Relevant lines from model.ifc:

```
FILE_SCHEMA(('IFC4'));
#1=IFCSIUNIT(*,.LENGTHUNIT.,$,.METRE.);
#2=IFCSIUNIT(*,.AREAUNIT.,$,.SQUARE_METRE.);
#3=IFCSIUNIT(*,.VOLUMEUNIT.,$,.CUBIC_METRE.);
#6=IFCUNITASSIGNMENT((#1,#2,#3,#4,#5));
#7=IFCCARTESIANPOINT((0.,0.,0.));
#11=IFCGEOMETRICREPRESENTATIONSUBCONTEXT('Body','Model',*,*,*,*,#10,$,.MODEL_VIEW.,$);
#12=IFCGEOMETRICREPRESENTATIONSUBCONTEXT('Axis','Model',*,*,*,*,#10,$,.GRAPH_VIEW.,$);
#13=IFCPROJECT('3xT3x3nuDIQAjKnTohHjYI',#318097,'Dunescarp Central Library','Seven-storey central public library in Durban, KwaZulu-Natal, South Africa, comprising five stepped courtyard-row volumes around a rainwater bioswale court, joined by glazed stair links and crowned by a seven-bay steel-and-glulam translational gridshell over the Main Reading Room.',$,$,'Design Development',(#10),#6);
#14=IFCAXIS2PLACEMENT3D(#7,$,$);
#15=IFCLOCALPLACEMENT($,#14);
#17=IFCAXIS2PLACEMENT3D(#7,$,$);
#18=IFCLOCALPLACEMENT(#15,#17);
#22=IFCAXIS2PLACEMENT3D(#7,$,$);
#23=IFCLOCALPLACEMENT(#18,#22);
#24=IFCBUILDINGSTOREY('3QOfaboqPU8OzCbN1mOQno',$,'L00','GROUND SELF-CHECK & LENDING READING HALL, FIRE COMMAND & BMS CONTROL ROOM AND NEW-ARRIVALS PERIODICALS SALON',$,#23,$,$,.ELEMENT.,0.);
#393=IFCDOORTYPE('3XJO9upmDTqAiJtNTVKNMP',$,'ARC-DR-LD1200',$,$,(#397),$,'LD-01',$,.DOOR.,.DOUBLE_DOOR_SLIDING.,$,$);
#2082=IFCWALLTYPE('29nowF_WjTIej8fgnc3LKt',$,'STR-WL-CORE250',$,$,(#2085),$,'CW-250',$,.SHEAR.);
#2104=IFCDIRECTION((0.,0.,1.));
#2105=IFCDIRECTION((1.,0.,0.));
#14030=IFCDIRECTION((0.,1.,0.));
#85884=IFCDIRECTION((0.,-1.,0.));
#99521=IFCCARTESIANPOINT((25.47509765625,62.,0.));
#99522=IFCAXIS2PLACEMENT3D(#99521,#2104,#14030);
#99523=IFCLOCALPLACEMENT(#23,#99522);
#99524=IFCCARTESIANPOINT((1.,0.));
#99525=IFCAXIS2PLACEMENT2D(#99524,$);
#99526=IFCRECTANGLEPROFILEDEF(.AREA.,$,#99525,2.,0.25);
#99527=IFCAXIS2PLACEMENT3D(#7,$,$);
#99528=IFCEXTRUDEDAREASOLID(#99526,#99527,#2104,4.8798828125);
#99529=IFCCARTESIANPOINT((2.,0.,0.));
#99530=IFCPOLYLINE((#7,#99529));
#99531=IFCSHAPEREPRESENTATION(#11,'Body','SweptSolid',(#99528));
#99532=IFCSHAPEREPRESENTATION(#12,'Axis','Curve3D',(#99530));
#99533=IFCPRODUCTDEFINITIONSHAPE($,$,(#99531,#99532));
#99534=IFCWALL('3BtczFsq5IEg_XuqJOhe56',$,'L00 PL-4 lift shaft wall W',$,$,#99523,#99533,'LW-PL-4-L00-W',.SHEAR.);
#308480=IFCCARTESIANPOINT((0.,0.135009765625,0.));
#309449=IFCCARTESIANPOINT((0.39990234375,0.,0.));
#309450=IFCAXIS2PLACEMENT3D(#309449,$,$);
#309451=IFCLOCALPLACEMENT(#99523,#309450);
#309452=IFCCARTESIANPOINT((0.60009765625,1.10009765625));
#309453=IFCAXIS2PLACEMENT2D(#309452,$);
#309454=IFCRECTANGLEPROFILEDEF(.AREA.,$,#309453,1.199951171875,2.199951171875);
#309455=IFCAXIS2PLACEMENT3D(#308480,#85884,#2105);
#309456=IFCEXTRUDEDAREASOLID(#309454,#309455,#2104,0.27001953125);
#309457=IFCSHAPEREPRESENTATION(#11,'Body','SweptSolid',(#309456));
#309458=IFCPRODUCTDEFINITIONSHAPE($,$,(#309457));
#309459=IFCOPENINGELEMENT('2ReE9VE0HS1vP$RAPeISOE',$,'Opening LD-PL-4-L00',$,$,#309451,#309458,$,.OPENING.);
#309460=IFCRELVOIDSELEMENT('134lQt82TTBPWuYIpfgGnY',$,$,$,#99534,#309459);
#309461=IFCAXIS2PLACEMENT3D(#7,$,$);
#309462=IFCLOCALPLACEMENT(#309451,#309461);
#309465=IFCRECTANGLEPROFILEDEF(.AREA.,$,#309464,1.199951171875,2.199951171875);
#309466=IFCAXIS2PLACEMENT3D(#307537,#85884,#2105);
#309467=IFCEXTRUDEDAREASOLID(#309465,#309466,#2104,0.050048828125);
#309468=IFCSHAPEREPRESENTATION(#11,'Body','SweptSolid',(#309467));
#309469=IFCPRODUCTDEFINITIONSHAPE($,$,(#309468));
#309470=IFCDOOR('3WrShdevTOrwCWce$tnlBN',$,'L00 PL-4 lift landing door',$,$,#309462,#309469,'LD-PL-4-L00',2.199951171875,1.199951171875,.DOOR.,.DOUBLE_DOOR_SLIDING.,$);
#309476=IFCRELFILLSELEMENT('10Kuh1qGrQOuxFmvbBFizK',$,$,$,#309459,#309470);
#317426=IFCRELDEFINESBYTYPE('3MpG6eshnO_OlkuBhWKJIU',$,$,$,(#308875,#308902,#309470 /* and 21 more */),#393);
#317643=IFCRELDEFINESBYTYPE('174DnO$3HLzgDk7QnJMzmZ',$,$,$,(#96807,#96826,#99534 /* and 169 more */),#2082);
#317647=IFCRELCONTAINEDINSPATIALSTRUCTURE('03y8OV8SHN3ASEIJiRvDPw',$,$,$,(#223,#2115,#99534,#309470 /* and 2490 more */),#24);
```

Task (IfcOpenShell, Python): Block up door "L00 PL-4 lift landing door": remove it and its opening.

```python
import ifcopenshell
import ifcopenshell.api.feature
import ifcopenshell.api.root
import ifcopenshell.geom
import ifcopenshell.util.shape

model = ifcopenshell.open("model.ifc")
settings = ifcopenshell.geom.settings()


def volume(element):
    """Net volume in cubic metres, openings subtracted."""
    shape = ifcopenshell.geom.create_shape(settings, element)
    return ifcopenshell.util.shape.get_volume(shape.geometry)


door = model.by_guid("3WrShdevTOrwCWce$tnlBN")
opening = door.FillsVoids[0].RelatingOpeningElement
wall = opening.VoidsElements[0].RelatingBuildingElement
before = volume(wall)

ifcopenshell.api.root.remove_product(model, product=door)
ifcopenshell.api.feature.remove_feature(model, feature=opening)

after = volume(wall)

print(f"wall volume {before:.3f} -> {after:.3f} m3")

model.write("model_rev.ifc")
```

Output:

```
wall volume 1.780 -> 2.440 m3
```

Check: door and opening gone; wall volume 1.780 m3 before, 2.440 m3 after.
